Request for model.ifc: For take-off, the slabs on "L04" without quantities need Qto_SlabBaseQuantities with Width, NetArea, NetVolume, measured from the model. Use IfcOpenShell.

First a look at what the model holds.

```python
import ifcopenshell
import ifcopenshell.util.element
import ifcopenshell.util.unit

model = ifcopenshell.open("model.ifc")
print(model.schema)
for unit_type in ("LENGTHUNIT", "AREAUNIT", "VOLUMEUNIT"):
    print(unit_type, ifcopenshell.util.unit.calculate_unit_scale(model, unit_type))
storey = next(s for s in model.by_type("IfcBuildingStorey") if s.Name == "L04")
slabs = [e for e in ifcopenshell.util.element.get_decomposition(storey) if e.is_a("IfcSlab")]
for e in sorted(slabs, key=lambda e: e.id()):
    print(e.id(), e.is_a(), e.Name, list(ifcopenshell.util.element.get_psets(e, qtos_only=True)), sep=" | ")
```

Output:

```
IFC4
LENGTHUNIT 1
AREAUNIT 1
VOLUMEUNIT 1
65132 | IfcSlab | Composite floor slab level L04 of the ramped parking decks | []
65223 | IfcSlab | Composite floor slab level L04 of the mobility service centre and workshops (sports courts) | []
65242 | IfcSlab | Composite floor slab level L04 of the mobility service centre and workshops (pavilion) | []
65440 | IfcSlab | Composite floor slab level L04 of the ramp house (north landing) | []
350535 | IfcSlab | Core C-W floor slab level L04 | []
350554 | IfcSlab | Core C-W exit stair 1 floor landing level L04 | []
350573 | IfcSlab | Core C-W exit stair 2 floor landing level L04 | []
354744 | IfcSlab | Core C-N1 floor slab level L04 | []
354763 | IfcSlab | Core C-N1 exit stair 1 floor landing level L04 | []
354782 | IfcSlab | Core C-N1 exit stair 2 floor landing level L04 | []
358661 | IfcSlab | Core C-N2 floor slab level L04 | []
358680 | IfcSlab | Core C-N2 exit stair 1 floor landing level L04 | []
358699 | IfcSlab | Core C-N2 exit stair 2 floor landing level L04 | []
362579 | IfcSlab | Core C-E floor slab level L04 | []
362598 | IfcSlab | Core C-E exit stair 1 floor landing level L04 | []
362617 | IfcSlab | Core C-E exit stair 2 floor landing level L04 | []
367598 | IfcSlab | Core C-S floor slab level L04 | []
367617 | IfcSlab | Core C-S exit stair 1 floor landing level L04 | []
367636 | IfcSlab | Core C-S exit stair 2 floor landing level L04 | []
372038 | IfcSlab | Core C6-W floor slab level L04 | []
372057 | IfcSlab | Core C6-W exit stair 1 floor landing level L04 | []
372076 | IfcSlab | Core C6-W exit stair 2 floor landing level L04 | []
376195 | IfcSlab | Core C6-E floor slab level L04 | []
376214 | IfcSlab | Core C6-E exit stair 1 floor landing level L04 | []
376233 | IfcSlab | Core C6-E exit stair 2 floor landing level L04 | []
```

```python
import ifcopenshell
import ifcopenshell.api.pset
import ifcopenshell.geom
import ifcopenshell.util.element
import ifcopenshell.util.shape
import ifcopenshell.util.unit

model = ifcopenshell.open("model.ifc")
unit_scale = ifcopenshell.util.unit.calculate_unit_scale(model)
area_scale = ifcopenshell.util.unit.calculate_unit_scale(model, "AREAUNIT")
volume_scale = ifcopenshell.util.unit.calculate_unit_scale(model, "VOLUMEUNIT")
settings = ifcopenshell.geom.settings()

storey = next(s for s in model.by_type("IfcBuildingStorey") if s.Name == "L04")
slabs = [e for e in ifcopenshell.util.element.get_decomposition(storey) if e.is_a("IfcSlab")]

for e in sorted(slabs, key=lambda e: e.id()):
    if ifcopenshell.util.element.get_psets(e, qtos_only=True, should_inherit=False):
        continue
    # Geometry comes back in metres, in the element's own axes.
    shape = ifcopenshell.geom.create_shape(settings, e)
    values = {
        "Width": ifcopenshell.util.shape.get_z(shape.geometry) / unit_scale,
        "NetArea": ifcopenshell.util.shape.get_footprint_area(shape.geometry) / area_scale,
        "NetVolume": ifcopenshell.util.shape.get_volume(shape.geometry) / volume_scale,
    }
    qto = ifcopenshell.api.pset.add_qto(model, product=e, name="Qto_SlabBaseQuantities")
    ifcopenshell.api.pset.edit_qto(model, qto=qto, properties=values)
    print(e.id(), {k: round(v, 3) for k, v in values.items()})

model.write("model_rev.ifc")
```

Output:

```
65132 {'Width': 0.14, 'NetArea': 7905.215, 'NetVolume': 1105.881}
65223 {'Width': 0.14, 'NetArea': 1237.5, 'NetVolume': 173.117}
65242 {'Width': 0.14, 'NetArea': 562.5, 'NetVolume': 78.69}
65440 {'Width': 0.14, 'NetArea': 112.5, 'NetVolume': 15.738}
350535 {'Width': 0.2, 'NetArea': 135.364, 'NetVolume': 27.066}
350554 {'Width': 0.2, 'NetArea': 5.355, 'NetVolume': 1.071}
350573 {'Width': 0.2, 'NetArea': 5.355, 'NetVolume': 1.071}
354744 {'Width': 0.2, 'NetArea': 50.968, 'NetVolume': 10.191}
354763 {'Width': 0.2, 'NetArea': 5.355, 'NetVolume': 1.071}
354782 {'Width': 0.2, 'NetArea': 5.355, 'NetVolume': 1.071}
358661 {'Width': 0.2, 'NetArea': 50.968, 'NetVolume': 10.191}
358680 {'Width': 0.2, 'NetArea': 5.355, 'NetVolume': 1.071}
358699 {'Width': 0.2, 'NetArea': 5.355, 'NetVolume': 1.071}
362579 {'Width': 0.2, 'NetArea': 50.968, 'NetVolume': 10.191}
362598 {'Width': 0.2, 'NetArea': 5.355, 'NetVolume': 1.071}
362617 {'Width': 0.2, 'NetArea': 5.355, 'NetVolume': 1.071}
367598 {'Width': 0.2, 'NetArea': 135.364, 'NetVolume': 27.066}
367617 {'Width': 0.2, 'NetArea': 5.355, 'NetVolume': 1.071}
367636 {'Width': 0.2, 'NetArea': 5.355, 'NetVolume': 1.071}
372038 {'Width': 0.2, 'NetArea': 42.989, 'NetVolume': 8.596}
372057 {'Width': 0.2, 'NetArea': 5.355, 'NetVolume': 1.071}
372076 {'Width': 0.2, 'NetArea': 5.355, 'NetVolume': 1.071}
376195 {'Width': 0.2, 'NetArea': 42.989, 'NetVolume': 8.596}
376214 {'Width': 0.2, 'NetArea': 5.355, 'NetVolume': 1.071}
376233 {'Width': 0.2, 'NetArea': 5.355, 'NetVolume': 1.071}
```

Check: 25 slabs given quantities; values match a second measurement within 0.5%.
